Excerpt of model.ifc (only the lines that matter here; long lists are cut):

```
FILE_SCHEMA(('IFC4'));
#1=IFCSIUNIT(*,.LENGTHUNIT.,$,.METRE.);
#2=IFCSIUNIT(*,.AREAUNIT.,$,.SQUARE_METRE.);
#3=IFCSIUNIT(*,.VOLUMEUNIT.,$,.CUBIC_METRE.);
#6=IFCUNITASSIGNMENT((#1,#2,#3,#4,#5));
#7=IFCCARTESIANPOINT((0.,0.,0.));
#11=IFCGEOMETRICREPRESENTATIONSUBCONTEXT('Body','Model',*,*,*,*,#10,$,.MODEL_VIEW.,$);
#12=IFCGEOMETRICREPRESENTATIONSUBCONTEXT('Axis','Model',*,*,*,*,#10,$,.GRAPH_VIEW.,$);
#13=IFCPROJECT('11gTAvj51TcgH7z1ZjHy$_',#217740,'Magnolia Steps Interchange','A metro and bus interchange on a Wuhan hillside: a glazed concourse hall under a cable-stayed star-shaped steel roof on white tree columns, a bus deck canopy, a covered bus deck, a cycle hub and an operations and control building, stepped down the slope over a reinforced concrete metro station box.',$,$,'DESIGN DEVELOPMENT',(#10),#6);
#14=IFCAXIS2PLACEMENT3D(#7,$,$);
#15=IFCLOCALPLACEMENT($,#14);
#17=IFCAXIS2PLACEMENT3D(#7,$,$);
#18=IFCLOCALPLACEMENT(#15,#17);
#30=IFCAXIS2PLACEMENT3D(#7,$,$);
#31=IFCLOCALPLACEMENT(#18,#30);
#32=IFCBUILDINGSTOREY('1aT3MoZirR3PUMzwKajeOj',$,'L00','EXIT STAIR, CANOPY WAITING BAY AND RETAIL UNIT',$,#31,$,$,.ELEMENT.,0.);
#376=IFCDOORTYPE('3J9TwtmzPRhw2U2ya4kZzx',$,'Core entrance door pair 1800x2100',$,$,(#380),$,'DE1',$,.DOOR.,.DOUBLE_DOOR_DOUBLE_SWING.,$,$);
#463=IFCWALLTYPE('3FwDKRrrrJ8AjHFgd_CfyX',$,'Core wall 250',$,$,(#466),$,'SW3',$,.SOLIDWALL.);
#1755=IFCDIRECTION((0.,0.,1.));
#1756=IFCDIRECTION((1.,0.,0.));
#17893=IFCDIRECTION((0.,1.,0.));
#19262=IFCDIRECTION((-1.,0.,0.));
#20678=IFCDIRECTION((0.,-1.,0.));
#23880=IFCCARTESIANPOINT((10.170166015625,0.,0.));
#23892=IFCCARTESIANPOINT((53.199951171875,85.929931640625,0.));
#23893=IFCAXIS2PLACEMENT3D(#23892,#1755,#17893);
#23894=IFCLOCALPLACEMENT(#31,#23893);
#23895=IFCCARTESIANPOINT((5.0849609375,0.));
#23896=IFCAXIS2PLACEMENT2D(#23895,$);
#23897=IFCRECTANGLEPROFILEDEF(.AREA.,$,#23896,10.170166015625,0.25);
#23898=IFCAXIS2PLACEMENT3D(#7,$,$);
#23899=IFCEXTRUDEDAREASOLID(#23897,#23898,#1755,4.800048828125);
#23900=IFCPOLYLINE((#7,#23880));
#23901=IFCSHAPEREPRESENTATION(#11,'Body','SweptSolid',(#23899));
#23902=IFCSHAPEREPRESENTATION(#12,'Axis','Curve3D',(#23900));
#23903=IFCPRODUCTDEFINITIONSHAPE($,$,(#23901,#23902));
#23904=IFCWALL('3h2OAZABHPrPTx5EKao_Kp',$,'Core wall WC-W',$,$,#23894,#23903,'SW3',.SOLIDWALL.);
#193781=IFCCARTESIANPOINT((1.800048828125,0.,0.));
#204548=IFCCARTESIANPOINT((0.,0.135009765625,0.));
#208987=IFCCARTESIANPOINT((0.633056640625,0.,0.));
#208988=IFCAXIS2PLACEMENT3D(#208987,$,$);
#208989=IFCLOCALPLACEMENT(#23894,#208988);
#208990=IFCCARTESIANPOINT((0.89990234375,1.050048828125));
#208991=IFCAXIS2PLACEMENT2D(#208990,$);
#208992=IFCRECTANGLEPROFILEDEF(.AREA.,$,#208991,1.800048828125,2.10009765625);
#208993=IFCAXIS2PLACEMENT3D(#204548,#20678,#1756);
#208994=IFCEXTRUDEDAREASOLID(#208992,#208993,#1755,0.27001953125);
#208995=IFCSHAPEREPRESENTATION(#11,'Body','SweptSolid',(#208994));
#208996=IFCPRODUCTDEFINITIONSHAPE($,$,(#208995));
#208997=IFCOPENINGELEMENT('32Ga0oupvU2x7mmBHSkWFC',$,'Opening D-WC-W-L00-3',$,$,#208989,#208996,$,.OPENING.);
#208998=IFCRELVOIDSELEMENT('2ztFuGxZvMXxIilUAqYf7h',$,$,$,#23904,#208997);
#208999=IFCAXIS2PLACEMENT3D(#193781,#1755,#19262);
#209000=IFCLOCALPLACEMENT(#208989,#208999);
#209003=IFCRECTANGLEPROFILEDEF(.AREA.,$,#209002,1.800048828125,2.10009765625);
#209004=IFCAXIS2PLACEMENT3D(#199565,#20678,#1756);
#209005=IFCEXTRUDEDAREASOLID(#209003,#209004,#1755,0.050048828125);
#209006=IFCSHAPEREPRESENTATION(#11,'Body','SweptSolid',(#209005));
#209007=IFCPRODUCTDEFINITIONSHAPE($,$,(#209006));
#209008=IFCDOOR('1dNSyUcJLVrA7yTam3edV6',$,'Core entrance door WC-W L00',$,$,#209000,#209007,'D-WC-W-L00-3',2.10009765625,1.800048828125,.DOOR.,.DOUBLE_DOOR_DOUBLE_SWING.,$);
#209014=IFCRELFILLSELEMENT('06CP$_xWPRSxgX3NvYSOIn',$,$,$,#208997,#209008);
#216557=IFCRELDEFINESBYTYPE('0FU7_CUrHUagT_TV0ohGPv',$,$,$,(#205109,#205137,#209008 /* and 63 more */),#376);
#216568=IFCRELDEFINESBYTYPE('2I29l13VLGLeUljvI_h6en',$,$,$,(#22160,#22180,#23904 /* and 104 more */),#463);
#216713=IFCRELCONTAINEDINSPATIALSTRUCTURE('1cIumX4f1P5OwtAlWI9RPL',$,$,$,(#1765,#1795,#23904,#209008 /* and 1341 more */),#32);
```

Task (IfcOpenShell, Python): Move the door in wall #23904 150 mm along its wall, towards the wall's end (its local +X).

```python
import ifcopenshell
import ifcopenshell.api.geometry
import ifcopenshell.util.placement

model = ifcopenshell.open("model.ifc")

door = model.by_id(209008)
opening = door.FillsVoids[0].RelatingOpeningElement
wall = opening.VoidsElements[0].RelatingBuildingElement

wall_matrix = ifcopenshell.util.placement.get_local_placement(wall.ObjectPlacement)
shift = wall_matrix[:3, 0] * 0.15
before = ifcopenshell.util.placement.get_local_placement(door.ObjectPlacement)[:3, 3].copy()

# The door is placed relative to its opening, so it follows when the opening moves.
matrix = ifcopenshell.util.placement.get_local_placement(opening.ObjectPlacement)
matrix[:3, 3] += shift
ifcopenshell.api.geometry.edit_object_placement(
    model, product=opening, matrix=matrix, is_si=False, should_transform_children=True
)

after = ifcopenshell.util.placement.get_local_placement(door.ObjectPlacement)[:3, 3]
print("door moved by", (after - before).round(3) + 0.0)

model.write("model_updated.ifc")
```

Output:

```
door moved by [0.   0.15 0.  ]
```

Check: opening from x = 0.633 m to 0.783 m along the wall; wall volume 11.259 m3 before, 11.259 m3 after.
